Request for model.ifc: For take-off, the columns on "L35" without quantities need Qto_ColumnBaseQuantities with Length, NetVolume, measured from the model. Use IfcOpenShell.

First a look at what the model holds.

```python
import ifcopenshell
import ifcopenshell.util.element
import ifcopenshell.util.unit

model = ifcopenshell.open("model.ifc")
print(model.schema)
for unit_type in ("LENGTHUNIT", "AREAUNIT", "VOLUMEUNIT"):
    print(unit_type, ifcopenshell.util.unit.calculate_unit_scale(model, unit_type))
storey = next(s for s in model.by_type("IfcBuildingStorey") if s.Name == "L35")
columns = [e for e in ifcopenshell.util.element.get_decomposition(storey) if e.is_a("IfcColumn")]
for e in sorted(columns, key=lambda e: e.id()):
    print(e.id(), e.is_a(), e.Name, list(ifcopenshell.util.element.get_psets(e, qtos_only=True)), sep=" | ")
```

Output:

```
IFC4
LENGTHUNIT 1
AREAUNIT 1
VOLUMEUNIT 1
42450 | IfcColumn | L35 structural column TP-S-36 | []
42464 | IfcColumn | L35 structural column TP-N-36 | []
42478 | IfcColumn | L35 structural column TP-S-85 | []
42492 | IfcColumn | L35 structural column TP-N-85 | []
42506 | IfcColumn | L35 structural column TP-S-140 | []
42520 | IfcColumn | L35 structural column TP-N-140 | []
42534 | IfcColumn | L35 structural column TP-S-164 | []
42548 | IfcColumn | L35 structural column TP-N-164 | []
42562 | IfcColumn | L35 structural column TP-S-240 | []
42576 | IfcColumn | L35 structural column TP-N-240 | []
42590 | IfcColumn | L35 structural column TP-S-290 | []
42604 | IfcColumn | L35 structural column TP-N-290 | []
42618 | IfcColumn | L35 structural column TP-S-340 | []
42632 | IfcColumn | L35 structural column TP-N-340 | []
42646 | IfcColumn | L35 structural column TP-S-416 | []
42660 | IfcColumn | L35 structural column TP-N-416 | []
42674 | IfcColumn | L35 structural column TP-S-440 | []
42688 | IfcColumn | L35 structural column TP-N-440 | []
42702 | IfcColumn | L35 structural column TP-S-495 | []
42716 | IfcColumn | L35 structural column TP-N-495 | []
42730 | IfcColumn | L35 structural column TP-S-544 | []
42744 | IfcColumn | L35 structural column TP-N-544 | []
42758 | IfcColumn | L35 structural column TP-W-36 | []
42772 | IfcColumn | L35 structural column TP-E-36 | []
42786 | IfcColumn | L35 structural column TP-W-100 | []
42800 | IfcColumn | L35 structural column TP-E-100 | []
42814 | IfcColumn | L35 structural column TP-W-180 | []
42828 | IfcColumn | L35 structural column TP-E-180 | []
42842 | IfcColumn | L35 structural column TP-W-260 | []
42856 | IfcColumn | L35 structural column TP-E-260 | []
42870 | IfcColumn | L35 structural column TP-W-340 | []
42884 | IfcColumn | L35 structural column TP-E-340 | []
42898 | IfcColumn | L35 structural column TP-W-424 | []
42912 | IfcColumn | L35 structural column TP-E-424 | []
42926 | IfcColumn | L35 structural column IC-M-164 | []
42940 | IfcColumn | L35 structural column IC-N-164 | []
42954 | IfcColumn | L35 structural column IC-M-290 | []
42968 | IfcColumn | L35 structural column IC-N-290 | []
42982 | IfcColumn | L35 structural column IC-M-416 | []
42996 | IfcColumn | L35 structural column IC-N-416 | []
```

```python
import ifcopenshell
import ifcopenshell.api.pset
import ifcopenshell.geom
import ifcopenshell.util.element
import ifcopenshell.util.shape
import ifcopenshell.util.unit

model = ifcopenshell.open("model.ifc")
unit_scale = ifcopenshell.util.unit.calculate_unit_scale(model)
volume_scale = ifcopenshell.util.unit.calculate_unit_scale(model, "VOLUMEUNIT")
settings = ifcopenshell.geom.settings()

storey = next(s for s in model.by_type("IfcBuildingStorey") if s.Name == "L35")
columns = [e for e in ifcopenshell.util.element.get_decomposition(storey) if e.is_a("IfcColumn")]

for e in sorted(columns, key=lambda e: e.id()):
    if ifcopenshell.util.element.get_psets(e, qtos_only=True, should_inherit=False):
        continue
    # Geometry comes back in metres, in the element's own axes.
    shape = ifcopenshell.geom.create_shape(settings, e)
    values = {
        "Length": ifcopenshell.util.shape.get_z(shape.geometry) / unit_scale,
        "NetVolume": ifcopenshell.util.shape.get_volume(shape.geometry) / volume_scale,
    }
    qto = ifcopenshell.api.pset.add_qto(model, product=e, name="Qto_ColumnBaseQuantities")
    ifcopenshell.api.pset.edit_qto(model, qto=qto, properties=values)
    print(e.id(), {k: round(v, 3) for k, v in values.items()})

model.write("model_updated.ifc")
```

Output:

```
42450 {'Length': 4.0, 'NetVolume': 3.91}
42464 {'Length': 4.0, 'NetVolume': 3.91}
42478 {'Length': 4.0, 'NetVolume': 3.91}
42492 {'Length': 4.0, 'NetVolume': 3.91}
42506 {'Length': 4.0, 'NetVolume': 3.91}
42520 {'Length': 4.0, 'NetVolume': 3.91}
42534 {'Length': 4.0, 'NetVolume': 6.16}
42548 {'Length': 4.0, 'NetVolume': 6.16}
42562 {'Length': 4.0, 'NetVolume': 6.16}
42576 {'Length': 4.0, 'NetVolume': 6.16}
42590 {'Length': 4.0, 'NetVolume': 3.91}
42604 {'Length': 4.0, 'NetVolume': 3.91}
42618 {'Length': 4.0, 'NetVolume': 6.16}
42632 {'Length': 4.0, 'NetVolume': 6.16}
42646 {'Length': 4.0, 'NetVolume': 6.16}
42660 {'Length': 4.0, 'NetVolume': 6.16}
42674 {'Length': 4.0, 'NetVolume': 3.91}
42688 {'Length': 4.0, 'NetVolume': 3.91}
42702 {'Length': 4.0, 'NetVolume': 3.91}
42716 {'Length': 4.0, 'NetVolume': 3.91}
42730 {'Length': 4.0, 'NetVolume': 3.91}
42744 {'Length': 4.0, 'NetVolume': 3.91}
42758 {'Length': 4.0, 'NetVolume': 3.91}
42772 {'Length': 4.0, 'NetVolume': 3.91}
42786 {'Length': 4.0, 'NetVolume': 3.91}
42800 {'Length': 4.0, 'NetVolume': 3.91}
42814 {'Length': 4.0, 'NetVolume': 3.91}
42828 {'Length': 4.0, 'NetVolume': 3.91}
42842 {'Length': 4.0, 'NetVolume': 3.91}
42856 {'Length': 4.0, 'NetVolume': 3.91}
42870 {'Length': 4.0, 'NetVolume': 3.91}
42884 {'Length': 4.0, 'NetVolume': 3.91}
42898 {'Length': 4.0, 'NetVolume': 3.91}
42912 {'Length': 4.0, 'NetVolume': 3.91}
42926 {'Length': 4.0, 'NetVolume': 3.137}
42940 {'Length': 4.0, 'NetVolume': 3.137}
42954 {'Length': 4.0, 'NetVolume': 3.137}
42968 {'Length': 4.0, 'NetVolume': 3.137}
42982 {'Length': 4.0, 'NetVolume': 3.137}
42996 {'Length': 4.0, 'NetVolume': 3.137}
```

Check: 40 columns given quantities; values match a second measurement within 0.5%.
